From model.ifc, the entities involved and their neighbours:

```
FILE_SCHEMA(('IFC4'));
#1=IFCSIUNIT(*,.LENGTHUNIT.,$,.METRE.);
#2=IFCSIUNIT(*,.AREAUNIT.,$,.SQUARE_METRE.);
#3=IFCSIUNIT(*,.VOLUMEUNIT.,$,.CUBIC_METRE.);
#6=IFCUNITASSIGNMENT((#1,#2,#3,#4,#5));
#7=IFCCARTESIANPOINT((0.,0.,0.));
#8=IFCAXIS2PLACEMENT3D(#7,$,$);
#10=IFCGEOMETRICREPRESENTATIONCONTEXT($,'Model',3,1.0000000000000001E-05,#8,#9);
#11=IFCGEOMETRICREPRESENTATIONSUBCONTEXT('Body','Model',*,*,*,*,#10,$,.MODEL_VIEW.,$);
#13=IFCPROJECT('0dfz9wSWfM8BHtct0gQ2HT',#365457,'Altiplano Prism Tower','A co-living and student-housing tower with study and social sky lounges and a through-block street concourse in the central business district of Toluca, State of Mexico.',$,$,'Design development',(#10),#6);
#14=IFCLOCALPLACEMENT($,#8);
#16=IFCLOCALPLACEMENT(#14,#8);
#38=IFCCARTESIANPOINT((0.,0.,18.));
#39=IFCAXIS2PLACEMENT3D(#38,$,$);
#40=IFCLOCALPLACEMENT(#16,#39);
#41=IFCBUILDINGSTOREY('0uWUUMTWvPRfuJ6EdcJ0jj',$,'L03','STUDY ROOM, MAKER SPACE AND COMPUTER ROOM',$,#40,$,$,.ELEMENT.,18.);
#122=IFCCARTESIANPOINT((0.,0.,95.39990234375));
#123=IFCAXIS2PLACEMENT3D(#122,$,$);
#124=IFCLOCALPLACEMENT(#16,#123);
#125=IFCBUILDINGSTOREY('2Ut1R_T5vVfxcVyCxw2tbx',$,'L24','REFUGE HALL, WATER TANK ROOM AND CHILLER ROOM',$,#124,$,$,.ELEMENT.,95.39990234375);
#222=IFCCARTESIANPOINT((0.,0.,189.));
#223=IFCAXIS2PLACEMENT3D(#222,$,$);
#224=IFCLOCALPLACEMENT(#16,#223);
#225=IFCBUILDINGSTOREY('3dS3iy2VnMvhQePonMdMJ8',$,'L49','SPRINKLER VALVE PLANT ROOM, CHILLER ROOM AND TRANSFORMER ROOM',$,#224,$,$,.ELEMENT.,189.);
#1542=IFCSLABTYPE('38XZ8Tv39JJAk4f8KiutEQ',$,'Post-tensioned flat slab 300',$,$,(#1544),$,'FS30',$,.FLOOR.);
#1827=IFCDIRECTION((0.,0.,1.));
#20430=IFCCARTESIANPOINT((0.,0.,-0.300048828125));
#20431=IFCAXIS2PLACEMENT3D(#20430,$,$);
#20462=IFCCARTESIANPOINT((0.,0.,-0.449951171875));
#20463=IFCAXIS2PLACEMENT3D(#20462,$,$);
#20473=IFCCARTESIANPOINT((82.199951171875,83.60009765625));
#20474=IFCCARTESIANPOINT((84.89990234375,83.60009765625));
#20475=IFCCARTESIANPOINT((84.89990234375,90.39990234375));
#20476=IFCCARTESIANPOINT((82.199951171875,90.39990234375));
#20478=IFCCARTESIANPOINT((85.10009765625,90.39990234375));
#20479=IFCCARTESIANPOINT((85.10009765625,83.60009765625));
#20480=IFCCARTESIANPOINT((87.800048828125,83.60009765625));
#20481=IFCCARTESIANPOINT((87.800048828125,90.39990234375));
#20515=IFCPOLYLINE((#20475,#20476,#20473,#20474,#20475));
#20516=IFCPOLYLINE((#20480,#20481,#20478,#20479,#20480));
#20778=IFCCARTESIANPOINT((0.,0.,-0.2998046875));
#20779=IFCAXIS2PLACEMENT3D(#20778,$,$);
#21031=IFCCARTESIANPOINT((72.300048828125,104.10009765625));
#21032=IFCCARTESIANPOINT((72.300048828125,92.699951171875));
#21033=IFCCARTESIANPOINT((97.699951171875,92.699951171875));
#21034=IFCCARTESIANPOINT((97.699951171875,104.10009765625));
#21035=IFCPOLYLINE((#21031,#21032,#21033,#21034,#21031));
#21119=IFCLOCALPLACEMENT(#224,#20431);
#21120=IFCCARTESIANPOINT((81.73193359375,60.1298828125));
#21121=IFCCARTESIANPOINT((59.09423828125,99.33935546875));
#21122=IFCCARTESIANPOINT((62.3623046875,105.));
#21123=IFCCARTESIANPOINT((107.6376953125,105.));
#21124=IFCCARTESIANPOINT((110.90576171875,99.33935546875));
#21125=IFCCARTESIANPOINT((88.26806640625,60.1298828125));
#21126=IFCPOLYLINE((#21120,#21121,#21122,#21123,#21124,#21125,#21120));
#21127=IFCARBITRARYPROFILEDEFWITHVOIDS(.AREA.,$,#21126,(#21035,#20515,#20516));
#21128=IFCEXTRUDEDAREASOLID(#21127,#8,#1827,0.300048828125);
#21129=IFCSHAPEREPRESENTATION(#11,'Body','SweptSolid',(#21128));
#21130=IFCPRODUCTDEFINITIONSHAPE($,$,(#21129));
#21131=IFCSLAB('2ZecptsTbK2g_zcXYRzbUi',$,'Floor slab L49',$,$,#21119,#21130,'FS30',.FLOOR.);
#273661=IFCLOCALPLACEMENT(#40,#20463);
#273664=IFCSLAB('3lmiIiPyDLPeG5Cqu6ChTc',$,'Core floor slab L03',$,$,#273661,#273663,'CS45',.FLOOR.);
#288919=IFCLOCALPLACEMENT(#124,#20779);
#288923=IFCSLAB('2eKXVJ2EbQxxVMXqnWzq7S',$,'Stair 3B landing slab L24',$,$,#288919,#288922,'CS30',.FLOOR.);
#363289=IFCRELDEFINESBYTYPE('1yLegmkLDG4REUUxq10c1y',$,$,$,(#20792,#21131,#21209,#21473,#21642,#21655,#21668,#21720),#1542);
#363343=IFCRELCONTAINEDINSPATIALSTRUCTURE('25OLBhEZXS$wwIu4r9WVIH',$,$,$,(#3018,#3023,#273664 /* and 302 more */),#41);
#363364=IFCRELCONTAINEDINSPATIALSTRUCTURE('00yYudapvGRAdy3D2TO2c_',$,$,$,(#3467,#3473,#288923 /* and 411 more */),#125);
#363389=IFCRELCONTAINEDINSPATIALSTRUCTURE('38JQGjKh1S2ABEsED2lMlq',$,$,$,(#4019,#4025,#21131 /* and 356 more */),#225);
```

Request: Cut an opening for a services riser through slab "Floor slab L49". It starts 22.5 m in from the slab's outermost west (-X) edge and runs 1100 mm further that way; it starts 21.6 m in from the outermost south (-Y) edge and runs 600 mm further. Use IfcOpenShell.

```python
import numpy as np
import ifcopenshell
import ifcopenshell.api.feature
import ifcopenshell.api.geometry
import ifcopenshell.api.root
import ifcopenshell.geom
import ifcopenshell.util.placement
import ifcopenshell.util.representation
import ifcopenshell.util.shape
import ifcopenshell.util.unit

model = ifcopenshell.open("model.ifc")
unit_scale = ifcopenshell.util.unit.calculate_unit_scale(model)
settings = ifcopenshell.geom.settings()


def volume(element):
    """Net volume in cubic metres, openings subtracted."""
    shape = ifcopenshell.geom.create_shape(settings, element)
    return ifcopenshell.util.shape.get_volume(shape.geometry)


slab = model.by_id(21131)
before = volume(slab)

# Extent in the slab's own axes, in metres. The edges named are its -X and -Y sides.
slab_shape = ifcopenshell.geom.create_shape(settings, slab)
vertices = ifcopenshell.util.shape.get_vertices(slab_shape.geometry)
x_min, y_min, bottom = vertices.min(axis=0)
top = vertices[:, 2].max()

opening = ifcopenshell.api.root.create_entity(model, ifc_class="IfcOpeningElement", name="Services riser opening", predefined_type="OPENING")
context = ifcopenshell.util.representation.get_context(model, "Model", "Body", "MODEL_VIEW")
width, depth = 1.1, 0.6
outline = [(0.0, 0.0), (width, 0.0), (width, depth), (0.0, depth), (0.0, 0.0)]
# Overshoot both faces by 50 mm so the cut is clean.
shape = ifcopenshell.api.geometry.add_slab_representation(
    model, context=context, depth=top - bottom + 0.1, polyline=outline
)
ifcopenshell.api.geometry.assign_representation(model, product=opening, representation=shape)

matrix = ifcopenshell.util.placement.get_local_placement(slab.ObjectPlacement)
matrix[:, 3] = matrix @ np.append(np.array([x_min + 22.5, y_min + 21.6, bottom - 0.05]) / unit_scale, 1.0)
ifcopenshell.api.geometry.edit_object_placement(model, product=opening, matrix=matrix, is_si=False)
ifcopenshell.api.feature.add_feature(model, feature=opening, element=slab)

after = volume(slab)

print(f"slab volume {before:.3f} -> {after:.3f} m3")

model.write("model_edited.ifc")
```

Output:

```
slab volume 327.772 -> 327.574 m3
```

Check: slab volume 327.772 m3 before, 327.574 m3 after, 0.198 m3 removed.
